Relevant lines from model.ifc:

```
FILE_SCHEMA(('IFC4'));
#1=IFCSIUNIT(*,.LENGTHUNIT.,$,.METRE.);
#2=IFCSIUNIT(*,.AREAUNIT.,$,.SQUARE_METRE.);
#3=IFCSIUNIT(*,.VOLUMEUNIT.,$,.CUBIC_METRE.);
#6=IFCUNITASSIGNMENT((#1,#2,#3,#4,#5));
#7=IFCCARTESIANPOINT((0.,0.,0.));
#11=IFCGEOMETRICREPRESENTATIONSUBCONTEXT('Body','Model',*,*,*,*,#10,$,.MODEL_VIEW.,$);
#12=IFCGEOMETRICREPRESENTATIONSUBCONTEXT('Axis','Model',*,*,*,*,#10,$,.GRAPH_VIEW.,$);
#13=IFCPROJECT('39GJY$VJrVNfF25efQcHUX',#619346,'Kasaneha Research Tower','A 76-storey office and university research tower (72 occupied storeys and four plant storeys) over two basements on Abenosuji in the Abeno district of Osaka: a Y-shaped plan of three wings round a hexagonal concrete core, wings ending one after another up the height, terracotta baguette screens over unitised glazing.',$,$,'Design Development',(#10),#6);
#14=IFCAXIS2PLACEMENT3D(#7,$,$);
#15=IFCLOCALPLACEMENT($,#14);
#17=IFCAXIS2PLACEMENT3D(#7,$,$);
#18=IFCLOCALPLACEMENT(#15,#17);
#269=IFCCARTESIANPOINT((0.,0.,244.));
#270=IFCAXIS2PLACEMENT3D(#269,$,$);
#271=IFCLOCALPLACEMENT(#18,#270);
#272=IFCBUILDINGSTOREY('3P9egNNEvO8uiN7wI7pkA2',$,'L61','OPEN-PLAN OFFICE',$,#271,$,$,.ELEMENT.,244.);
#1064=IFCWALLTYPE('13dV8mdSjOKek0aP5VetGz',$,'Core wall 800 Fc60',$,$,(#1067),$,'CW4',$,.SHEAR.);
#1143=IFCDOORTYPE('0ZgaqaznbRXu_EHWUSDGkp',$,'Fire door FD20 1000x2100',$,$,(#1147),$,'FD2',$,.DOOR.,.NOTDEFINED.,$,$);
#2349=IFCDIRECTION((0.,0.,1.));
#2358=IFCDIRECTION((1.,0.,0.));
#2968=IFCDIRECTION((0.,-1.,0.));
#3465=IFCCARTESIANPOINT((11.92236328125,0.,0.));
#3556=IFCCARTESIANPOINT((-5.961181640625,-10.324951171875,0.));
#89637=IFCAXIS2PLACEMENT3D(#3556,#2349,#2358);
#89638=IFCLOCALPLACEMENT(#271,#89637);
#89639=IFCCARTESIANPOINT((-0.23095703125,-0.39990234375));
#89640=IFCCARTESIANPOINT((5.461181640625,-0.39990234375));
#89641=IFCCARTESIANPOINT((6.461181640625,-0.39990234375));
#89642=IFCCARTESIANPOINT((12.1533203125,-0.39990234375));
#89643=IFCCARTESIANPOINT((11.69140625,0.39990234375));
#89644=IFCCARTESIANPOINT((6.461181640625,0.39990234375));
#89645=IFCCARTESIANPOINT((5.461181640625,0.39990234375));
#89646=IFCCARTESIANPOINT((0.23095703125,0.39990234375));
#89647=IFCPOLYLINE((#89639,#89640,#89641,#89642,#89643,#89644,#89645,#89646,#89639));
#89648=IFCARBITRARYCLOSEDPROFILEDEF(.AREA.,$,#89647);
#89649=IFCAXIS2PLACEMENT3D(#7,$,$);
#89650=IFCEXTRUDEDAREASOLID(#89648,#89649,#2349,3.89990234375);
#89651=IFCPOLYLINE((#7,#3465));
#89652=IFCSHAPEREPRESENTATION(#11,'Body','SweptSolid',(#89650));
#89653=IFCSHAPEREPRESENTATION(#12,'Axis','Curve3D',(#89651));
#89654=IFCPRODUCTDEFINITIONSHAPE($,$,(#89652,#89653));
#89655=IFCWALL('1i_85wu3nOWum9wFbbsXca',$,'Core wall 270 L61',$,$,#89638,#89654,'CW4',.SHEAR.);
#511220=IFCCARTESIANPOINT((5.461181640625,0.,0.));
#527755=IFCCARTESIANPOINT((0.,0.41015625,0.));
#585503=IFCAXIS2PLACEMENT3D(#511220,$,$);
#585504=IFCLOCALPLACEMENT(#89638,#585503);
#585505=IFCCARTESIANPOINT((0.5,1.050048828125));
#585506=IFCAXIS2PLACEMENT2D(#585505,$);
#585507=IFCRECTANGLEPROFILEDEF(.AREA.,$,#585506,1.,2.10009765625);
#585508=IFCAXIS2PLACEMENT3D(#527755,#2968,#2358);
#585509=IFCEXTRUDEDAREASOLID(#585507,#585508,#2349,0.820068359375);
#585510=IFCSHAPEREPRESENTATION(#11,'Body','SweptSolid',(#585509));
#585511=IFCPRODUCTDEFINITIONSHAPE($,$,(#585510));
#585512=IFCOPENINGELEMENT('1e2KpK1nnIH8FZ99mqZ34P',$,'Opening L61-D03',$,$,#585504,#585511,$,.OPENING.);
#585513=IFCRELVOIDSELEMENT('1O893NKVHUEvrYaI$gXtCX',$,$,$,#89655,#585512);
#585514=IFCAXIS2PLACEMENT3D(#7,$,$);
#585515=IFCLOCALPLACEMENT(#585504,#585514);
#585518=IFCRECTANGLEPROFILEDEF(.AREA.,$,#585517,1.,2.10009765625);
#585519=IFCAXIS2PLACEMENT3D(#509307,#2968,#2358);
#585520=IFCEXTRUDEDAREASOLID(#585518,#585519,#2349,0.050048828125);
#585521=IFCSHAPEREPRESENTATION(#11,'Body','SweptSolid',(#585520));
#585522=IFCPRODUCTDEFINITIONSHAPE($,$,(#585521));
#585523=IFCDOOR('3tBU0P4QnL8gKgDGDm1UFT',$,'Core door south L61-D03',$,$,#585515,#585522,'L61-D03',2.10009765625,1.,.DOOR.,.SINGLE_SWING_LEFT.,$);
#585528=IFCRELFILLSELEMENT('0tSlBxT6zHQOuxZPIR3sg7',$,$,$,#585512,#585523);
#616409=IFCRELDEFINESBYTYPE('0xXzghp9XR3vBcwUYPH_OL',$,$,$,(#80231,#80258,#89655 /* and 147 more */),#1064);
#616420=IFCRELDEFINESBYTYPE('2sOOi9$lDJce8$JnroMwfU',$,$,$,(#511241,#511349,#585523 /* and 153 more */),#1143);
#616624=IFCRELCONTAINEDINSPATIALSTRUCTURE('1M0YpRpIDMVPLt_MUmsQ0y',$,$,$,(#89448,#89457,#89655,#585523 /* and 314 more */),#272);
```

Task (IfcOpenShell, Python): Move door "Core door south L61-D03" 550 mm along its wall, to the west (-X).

```python
import ifcopenshell
import ifcopenshell.api.geometry
import ifcopenshell.util.placement
import ifcopenshell.util.unit

model = ifcopenshell.open("model.ifc")
unit_scale = ifcopenshell.util.unit.calculate_unit_scale(model)

door = model.by_guid("3tBU0P4QnL8gKgDGDm1UFT")
opening = door.FillsVoids[0].RelatingOpeningElement
wall = opening.VoidsElements[0].RelatingBuildingElement

wall_matrix = ifcopenshell.util.placement.get_local_placement(wall.ObjectPlacement)
shift = wall_matrix[:3, 0] * -0.55 / unit_scale
before = ifcopenshell.util.placement.get_local_placement(door.ObjectPlacement)[:3, 3].copy()

# The door is placed relative to its opening, so it follows when the opening moves.
matrix = ifcopenshell.util.placement.get_local_placement(opening.ObjectPlacement)
matrix[:3, 3] += shift
ifcopenshell.api.geometry.edit_object_placement(
    model, product=opening, matrix=matrix, is_si=False, should_transform_children=True
)

after = ifcopenshell.util.placement.get_local_placement(door.ObjectPlacement)[:3, 3]
print("door moved by", (after - before).round(3) + 0.0)

model.write("model_v2.ifc")
```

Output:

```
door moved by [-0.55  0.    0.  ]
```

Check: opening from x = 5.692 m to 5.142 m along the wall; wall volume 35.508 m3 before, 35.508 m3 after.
